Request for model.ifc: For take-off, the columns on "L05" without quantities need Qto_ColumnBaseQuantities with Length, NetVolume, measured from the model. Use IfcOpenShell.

First a look at what the model holds.

```python
import ifcopenshell
import ifcopenshell.util.element
import ifcopenshell.util.unit

model = ifcopenshell.open("model.ifc")
print(model.schema)
for unit_type in ("LENGTHUNIT", "AREAUNIT", "VOLUMEUNIT"):
    print(unit_type, ifcopenshell.util.unit.calculate_unit_scale(model, unit_type))
storey = next(s for s in model.by_type("IfcBuildingStorey") if s.Name == "L05")
columns = [e for e in ifcopenshell.util.element.get_decomposition(storey) if e.is_a("IfcColumn")]
for e in sorted(columns, key=lambda e: e.id()):
    print(e.id(), e.is_a(), e.Name, list(ifcopenshell.util.element.get_psets(e, qtos_only=True)), sep=" | ")
```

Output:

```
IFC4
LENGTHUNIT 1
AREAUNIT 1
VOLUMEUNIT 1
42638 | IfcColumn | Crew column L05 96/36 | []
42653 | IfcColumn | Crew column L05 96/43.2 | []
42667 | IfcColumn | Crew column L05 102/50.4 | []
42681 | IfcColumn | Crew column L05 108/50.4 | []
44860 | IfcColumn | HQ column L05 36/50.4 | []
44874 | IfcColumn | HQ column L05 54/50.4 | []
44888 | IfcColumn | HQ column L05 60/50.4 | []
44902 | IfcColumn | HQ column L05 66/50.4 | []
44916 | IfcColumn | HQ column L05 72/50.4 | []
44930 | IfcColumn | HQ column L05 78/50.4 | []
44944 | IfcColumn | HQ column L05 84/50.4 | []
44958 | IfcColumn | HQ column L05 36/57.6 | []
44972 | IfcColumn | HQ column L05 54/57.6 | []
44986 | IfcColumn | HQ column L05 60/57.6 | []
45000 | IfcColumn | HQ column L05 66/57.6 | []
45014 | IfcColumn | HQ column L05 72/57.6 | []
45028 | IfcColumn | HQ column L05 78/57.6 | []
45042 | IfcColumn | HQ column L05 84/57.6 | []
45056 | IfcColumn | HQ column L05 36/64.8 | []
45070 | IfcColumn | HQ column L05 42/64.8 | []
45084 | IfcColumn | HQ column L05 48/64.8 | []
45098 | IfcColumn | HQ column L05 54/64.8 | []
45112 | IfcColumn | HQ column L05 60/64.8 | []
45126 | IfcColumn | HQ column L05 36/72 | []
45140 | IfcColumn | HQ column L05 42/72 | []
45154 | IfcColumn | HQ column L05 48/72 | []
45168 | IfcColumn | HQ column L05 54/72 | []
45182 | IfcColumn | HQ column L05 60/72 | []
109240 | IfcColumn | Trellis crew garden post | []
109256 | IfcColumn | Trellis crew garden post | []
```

```python
import ifcopenshell
import ifcopenshell.api.pset
import ifcopenshell.geom
import ifcopenshell.util.element
import ifcopenshell.util.shape
import ifcopenshell.util.unit

model = ifcopenshell.open("model.ifc")
unit_scale = ifcopenshell.util.unit.calculate_unit_scale(model)
volume_scale = ifcopenshell.util.unit.calculate_unit_scale(model, "VOLUMEUNIT")
settings = ifcopenshell.geom.settings()

storey = next(s for s in model.by_type("IfcBuildingStorey") if s.Name == "L05")
columns = [e for e in ifcopenshell.util.element.get_decomposition(storey) if e.is_a("IfcColumn")]

for e in sorted(columns, key=lambda e: e.id()):
    if ifcopenshell.util.element.get_psets(e, qtos_only=True, should_inherit=False):
        continue
    # Geometry comes back in metres, in the element's own axes.
    shape = ifcopenshell.geom.create_shape(settings, e)
    values = {
        "Length": ifcopenshell.util.shape.get_z(shape.geometry) / unit_scale,
        "NetVolume": ifcopenshell.util.shape.get_volume(shape.geometry) / volume_scale,
    }
    qto = ifcopenshell.api.pset.add_qto(model, product=e, name="Qto_ColumnBaseQuantities")
    ifcopenshell.api.pset.edit_qto(model, qto=qto, properties=values)
    print(e.id(), {k: round(v, 3) for k, v in values.items()})

model.write("model_edited.ifc")
```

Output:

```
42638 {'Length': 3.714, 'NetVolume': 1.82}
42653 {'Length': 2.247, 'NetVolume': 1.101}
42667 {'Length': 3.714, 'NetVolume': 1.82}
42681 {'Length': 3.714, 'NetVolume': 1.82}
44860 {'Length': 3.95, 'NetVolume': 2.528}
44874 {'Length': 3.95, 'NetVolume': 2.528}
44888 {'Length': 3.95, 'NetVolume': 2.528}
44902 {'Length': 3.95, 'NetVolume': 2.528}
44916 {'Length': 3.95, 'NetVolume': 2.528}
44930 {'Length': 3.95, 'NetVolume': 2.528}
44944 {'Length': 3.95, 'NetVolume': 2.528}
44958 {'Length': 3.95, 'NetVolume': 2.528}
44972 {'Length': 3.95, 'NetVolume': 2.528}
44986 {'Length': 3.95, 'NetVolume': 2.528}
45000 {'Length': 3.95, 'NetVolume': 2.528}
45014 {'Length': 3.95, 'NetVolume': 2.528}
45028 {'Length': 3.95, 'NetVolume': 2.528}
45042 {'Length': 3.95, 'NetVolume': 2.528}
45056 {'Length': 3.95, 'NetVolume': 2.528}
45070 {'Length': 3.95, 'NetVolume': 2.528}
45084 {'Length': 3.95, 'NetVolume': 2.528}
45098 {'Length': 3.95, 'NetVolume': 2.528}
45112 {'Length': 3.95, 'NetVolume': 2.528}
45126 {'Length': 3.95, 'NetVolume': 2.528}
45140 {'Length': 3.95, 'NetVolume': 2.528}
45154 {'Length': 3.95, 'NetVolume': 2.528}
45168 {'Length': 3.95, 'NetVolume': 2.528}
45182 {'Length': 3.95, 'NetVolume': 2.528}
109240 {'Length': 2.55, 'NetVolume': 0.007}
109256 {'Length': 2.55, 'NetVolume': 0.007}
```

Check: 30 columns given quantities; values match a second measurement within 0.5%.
